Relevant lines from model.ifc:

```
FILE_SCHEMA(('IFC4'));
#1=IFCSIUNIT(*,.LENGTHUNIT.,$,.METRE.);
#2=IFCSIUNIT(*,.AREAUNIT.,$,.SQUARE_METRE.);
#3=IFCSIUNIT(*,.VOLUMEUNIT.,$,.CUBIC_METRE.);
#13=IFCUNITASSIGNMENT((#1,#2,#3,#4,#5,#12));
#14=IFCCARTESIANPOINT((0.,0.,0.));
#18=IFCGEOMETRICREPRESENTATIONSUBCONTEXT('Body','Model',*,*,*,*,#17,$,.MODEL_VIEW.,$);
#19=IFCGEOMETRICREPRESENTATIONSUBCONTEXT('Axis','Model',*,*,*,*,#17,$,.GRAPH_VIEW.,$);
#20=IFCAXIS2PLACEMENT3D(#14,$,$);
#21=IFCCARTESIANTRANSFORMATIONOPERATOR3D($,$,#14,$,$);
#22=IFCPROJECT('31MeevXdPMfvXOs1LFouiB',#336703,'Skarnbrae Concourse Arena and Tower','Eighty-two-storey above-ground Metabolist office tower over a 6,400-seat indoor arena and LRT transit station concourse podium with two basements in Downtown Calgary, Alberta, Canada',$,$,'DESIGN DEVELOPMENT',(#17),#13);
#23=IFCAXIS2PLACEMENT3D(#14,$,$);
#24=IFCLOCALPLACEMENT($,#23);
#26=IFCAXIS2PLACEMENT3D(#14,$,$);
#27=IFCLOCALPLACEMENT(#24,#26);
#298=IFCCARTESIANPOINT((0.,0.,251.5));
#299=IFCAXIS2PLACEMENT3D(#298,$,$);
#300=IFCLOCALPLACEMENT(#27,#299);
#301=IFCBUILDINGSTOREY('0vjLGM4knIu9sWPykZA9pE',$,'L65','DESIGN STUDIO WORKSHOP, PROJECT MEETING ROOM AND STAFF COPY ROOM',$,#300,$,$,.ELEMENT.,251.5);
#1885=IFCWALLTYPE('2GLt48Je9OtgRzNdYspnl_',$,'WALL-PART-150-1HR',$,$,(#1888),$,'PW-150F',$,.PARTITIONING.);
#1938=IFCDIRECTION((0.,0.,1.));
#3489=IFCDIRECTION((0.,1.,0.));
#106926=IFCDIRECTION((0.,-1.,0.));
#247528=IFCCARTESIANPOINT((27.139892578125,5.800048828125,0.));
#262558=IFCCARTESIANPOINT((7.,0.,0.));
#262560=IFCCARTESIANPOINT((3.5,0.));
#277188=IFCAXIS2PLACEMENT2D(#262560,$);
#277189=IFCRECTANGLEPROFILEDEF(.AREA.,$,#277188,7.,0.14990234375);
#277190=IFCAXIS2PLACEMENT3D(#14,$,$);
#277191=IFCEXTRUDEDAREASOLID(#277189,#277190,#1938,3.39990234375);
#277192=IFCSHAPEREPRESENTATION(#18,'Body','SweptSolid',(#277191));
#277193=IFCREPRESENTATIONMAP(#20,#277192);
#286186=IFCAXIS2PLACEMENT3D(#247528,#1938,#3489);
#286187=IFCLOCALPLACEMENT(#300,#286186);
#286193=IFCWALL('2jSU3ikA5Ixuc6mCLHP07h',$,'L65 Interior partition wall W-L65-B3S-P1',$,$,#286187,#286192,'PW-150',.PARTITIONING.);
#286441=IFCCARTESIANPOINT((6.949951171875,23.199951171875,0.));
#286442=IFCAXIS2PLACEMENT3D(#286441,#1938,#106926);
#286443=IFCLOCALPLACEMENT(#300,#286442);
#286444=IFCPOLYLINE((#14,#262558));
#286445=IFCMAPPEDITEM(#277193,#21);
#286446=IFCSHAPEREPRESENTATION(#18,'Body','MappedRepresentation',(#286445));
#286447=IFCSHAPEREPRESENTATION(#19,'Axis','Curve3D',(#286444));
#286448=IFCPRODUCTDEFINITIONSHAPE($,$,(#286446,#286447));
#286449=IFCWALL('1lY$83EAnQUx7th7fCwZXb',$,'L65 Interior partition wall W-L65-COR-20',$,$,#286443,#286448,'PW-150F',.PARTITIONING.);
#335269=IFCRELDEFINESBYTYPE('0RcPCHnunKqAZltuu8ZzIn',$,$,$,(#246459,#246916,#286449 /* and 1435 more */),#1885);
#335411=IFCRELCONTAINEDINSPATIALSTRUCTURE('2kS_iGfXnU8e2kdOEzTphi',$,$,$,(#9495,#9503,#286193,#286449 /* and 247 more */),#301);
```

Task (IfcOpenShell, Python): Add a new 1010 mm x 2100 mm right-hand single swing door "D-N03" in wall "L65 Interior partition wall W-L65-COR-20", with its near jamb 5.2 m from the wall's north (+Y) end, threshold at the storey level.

```python
import numpy as np
import ifcopenshell
import ifcopenshell.api.feature
import ifcopenshell.api.geometry
import ifcopenshell.api.root
import ifcopenshell.api.spatial
import ifcopenshell.geom
import ifcopenshell.util.element
import ifcopenshell.util.placement
import ifcopenshell.util.representation
import ifcopenshell.util.shape
import ifcopenshell.util.unit

model = ifcopenshell.open("model.ifc")
unit_scale = ifcopenshell.util.unit.calculate_unit_scale(model)
settings = ifcopenshell.geom.settings()


def volume(element):
    """Net volume in cubic metres, openings subtracted."""
    shape = ifcopenshell.geom.create_shape(settings, element)
    return ifcopenshell.util.shape.get_volume(shape.geometry)


wall = model.by_id(286449)
storey = ifcopenshell.util.element.get_container(wall, ifc_class="IfcBuildingStorey")
context = ifcopenshell.util.representation.get_context(model, "Model", "Body", "MODEL_VIEW")
before = volume(wall)

width, height, from_end, sill = 1.01, 2.1, 5.2, 0.0  # metres

# The wall runs along its own X axis, and the end named is its -X end.
wall_shape = ifcopenshell.geom.create_shape(settings, wall)
x, y, z = ifcopenshell.util.shape.get_vertices(wall_shape.geometry).T
start = x.min() + from_end
face, thickness = float(y.min()), float(y.max() - y.min())
wall_matrix = ifcopenshell.util.placement.get_local_placement(wall.ObjectPlacement)
level = ifcopenshell.util.placement.get_local_placement(storey.ObjectPlacement)[2, 3]


def in_wall(x, y):
    """Placement at x, y metres in the wall's axes, at sill height."""
    matrix = wall_matrix.copy()
    matrix[:, 3] = wall_matrix @ np.array([x / unit_scale, y / unit_scale, 0.0, 1.0])
    matrix[2, 3] = level + sill / unit_scale
    return matrix


# Opening: a box that overshoots both wall faces by 50 mm.
opening = ifcopenshell.api.root.create_entity(model, ifc_class="IfcOpeningElement", predefined_type="OPENING")
box = ifcopenshell.api.geometry.add_wall_representation(
    model, context=context, length=width, height=height, thickness=thickness + 0.1
)
ifcopenshell.api.geometry.assign_representation(model, product=opening, representation=box)
ifcopenshell.api.geometry.edit_object_placement(model, product=opening, matrix=in_wall(start, face - 0.05), is_si=False)
ifcopenshell.api.feature.add_feature(model, feature=opening, element=wall)

door = ifcopenshell.api.root.create_entity(model, ifc_class="IfcDoor", name="D-N03", predefined_type="DOOR")
door.OverallWidth, door.OverallHeight = width / unit_scale, height / unit_scale
door.OperationType = "SINGLE_SWING_RIGHT"
body = ifcopenshell.api.geometry.add_door_representation(
    model,
    context=context,
    overall_width=door.OverallWidth,
    overall_height=door.OverallHeight,
    operation_type="SINGLE_SWING_RIGHT",
    lining_properties={"LiningDepth": thickness / unit_scale, "ThresholdDepth": thickness / unit_scale},
)
ifcopenshell.api.geometry.assign_representation(model, product=door, representation=body)
ifcopenshell.api.spatial.assign_container(model, products=[door], relating_structure=storey)
ifcopenshell.api.feature.add_filling(model, opening=opening, element=door)

# The lining spans the wall, so the door starts at the wall face.
ifcopenshell.api.geometry.edit_object_placement(model, product=door, matrix=in_wall(start, face), is_si=False)

after = volume(wall)

print(f"wall volume {before:.3f} -> {after:.3f} m3")

model.write("model-out.ifc")
```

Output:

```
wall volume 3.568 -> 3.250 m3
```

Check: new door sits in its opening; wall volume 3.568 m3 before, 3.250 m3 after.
